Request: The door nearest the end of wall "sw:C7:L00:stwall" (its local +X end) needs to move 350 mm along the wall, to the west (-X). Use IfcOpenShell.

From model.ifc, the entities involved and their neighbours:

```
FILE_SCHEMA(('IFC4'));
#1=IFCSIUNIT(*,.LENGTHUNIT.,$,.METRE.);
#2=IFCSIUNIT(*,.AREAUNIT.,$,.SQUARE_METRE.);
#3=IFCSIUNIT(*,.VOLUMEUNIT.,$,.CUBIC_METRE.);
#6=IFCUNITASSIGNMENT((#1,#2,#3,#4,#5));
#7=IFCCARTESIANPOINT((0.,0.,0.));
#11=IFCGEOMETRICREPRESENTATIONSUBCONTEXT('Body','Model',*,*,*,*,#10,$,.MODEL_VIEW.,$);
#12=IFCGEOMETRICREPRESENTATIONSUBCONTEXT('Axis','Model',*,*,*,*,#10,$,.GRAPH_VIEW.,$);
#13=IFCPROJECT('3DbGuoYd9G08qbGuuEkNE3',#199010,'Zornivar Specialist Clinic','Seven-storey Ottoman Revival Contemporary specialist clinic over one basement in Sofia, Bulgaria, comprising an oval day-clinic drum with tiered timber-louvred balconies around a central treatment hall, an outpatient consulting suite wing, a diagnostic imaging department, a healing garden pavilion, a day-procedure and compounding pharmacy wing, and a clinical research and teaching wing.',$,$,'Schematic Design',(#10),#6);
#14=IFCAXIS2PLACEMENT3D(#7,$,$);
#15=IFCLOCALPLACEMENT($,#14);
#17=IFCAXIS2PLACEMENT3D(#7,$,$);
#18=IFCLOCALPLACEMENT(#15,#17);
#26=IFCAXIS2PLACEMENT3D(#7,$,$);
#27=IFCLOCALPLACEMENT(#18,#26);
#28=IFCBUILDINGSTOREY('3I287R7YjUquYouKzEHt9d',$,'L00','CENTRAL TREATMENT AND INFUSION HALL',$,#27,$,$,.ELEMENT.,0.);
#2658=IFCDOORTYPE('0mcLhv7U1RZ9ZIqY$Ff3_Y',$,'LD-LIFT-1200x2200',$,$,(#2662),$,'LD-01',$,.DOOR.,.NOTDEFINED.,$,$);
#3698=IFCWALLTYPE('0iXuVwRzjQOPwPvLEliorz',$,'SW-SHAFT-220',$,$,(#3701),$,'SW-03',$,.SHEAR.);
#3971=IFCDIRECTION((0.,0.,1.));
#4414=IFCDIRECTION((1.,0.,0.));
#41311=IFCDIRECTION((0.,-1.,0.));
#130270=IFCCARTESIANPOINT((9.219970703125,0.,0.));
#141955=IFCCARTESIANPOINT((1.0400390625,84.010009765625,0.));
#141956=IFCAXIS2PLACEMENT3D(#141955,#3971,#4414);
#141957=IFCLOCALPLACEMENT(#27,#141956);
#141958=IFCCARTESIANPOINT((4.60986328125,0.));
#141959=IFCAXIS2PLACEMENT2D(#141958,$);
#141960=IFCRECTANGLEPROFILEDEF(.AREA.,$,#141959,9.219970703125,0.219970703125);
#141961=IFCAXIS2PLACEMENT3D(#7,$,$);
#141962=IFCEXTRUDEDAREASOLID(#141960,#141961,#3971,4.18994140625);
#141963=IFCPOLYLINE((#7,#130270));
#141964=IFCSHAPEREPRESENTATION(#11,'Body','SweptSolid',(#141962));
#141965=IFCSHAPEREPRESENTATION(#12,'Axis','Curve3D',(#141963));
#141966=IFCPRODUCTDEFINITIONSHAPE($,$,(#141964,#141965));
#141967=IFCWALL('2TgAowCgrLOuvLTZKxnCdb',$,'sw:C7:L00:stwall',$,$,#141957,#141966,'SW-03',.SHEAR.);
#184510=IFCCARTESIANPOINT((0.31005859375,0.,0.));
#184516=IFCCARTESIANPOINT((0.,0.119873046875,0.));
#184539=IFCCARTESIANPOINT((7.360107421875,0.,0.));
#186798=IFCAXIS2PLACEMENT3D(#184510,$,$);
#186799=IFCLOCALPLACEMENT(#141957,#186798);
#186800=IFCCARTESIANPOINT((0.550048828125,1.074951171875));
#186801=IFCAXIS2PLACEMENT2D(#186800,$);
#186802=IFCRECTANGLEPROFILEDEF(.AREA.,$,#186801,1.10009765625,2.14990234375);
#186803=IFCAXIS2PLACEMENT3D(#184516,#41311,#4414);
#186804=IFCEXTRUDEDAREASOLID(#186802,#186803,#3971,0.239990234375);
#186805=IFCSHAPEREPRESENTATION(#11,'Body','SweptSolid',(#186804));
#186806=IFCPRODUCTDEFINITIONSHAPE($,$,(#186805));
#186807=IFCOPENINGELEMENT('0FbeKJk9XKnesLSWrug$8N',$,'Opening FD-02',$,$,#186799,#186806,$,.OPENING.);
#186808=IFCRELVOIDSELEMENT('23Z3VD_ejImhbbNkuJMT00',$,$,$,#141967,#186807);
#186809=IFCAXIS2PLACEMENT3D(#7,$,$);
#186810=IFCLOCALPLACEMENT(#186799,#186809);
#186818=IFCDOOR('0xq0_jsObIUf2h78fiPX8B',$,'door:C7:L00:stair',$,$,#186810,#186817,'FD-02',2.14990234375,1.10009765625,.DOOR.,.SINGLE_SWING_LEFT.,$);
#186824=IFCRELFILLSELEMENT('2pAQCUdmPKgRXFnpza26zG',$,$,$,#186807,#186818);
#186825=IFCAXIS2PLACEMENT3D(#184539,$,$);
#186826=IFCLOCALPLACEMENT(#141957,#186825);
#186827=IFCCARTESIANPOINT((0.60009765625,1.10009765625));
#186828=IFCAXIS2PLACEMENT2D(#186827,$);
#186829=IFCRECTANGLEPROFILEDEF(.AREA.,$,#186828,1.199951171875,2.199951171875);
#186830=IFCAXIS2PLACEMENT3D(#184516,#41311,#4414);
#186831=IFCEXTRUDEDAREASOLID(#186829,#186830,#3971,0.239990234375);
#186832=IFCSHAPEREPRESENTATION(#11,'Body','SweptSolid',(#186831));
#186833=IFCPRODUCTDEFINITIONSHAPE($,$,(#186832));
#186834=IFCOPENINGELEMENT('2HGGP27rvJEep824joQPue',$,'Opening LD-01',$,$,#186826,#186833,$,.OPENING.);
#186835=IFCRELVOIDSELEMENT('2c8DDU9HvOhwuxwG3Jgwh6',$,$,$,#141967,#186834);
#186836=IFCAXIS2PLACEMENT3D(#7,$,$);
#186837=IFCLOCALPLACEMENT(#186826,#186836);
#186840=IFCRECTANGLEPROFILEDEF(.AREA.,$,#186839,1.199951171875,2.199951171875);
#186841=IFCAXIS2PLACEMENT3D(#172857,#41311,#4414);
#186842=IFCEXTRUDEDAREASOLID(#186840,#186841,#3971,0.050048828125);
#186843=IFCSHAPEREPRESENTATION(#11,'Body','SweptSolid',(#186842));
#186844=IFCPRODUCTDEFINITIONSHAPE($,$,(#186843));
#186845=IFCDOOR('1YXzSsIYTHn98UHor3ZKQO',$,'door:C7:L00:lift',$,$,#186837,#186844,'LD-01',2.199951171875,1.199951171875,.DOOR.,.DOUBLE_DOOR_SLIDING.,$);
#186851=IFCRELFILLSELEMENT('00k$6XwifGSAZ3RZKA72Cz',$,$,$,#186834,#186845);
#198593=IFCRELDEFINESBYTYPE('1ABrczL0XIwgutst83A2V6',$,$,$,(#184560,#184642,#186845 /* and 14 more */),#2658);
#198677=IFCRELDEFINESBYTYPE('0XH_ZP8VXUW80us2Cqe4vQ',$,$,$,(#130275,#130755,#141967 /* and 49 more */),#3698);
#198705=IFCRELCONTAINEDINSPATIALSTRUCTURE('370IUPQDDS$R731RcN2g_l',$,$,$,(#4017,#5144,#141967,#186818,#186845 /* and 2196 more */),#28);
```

```python
import ifcopenshell
import ifcopenshell.api.geometry
import ifcopenshell.util.placement

model = ifcopenshell.open("model.ifc")

door = model.by_guid("1YXzSsIYTHn98UHor3ZKQO")
opening = door.FillsVoids[0].RelatingOpeningElement
wall = opening.VoidsElements[0].RelatingBuildingElement

wall_matrix = ifcopenshell.util.placement.get_local_placement(wall.ObjectPlacement)
shift = wall_matrix[:3, 0] * -0.35
before = ifcopenshell.util.placement.get_local_placement(door.ObjectPlacement)[:3, 3].copy()

# The door is placed relative to its opening, so it follows when the opening moves.
matrix = ifcopenshell.util.placement.get_local_placement(opening.ObjectPlacement)
matrix[:3, 3] += shift
ifcopenshell.api.geometry.edit_object_placement(
    model, product=opening, matrix=matrix, is_si=False, should_transform_children=True
)

after = ifcopenshell.util.placement.get_local_placement(door.ObjectPlacement)[:3, 3]
print("door moved by", (after - before).round(3) + 0.0)

model.write("model-out.ifc")
```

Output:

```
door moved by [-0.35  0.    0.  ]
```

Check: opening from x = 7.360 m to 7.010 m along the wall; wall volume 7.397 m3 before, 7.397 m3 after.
